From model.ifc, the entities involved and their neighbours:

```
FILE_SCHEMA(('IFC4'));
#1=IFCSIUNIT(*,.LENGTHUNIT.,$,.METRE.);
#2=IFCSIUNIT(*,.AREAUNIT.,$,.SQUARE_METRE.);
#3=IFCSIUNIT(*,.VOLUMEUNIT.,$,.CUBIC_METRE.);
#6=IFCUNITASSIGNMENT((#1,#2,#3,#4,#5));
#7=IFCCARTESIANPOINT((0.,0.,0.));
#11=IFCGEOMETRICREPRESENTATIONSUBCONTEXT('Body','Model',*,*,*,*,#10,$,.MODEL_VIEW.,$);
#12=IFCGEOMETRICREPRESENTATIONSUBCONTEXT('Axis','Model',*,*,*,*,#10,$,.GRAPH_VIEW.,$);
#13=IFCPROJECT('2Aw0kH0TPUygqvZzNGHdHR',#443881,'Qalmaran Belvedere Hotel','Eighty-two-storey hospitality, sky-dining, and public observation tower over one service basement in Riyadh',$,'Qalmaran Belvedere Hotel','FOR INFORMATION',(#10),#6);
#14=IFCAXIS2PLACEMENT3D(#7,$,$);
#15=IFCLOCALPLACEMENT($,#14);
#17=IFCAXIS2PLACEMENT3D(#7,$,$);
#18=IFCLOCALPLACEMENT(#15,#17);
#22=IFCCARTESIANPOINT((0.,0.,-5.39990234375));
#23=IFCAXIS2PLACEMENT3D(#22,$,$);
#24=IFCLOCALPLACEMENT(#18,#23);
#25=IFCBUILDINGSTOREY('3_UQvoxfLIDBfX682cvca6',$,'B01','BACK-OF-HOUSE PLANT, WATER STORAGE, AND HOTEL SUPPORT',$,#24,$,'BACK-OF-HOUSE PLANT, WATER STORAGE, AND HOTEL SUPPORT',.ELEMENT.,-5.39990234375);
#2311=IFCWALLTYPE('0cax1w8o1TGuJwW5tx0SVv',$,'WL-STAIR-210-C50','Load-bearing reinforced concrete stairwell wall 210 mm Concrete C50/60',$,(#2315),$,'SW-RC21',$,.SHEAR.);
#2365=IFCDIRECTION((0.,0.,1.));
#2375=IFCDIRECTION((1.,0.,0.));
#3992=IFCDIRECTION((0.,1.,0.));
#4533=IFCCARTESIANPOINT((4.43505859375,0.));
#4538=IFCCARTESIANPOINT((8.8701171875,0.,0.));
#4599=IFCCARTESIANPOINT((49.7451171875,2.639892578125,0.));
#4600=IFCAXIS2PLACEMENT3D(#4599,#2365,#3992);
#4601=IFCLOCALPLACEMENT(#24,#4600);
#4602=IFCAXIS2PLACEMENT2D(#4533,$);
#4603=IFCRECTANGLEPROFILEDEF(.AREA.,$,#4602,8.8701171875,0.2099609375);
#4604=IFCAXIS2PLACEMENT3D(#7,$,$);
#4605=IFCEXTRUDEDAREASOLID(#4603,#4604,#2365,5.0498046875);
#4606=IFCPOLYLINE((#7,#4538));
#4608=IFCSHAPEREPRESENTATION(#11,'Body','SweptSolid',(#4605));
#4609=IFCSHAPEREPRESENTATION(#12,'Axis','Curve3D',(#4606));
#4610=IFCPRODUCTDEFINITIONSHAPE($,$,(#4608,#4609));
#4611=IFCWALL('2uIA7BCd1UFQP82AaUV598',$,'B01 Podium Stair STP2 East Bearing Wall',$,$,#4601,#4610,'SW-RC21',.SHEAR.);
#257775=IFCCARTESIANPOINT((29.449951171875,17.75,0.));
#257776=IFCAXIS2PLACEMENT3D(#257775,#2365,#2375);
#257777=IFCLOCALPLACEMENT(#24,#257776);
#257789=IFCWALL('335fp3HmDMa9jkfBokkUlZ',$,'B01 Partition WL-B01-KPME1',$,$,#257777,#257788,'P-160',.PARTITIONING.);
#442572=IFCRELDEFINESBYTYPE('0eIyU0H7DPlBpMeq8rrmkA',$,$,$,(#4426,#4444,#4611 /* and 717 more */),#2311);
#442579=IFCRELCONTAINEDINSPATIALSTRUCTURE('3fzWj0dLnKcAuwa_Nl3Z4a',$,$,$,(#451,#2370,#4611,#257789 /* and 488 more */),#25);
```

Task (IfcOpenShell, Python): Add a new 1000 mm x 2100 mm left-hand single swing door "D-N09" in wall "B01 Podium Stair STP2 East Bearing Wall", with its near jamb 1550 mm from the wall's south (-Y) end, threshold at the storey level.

```python
import numpy as np
import ifcopenshell
import ifcopenshell.api.feature
import ifcopenshell.api.geometry
import ifcopenshell.api.root
import ifcopenshell.api.spatial
import ifcopenshell.geom
import ifcopenshell.util.element
import ifcopenshell.util.placement
import ifcopenshell.util.representation
import ifcopenshell.util.shape
import ifcopenshell.util.unit

model = ifcopenshell.open("model.ifc")
unit_scale = ifcopenshell.util.unit.calculate_unit_scale(model)
settings = ifcopenshell.geom.settings()


def volume(element):
    """Net volume in cubic metres, openings subtracted."""
    shape = ifcopenshell.geom.create_shape(settings, element)
    return ifcopenshell.util.shape.get_volume(shape.geometry)


wall = model.by_guid("2uIA7BCd1UFQP82AaUV598")
storey = ifcopenshell.util.element.get_container(wall, ifc_class="IfcBuildingStorey")
context = ifcopenshell.util.representation.get_context(model, "Model", "Body", "MODEL_VIEW")
before = volume(wall)

width, height, from_end, sill = 1, 2.1, 1.55, 0.0  # metres

# The wall runs along its own X axis, and the end named is its -X end.
wall_shape = ifcopenshell.geom.create_shape(settings, wall)
x, y, z = ifcopenshell.util.shape.get_vertices(wall_shape.geometry).T
start = x.min() + from_end
face, thickness = float(y.min()), float(y.max() - y.min())
wall_matrix = ifcopenshell.util.placement.get_local_placement(wall.ObjectPlacement)
level = ifcopenshell.util.placement.get_local_placement(storey.ObjectPlacement)[2, 3]


def in_wall(x, y):
    """Placement at x, y metres in the wall's axes, at sill height."""
    matrix = wall_matrix.copy()
    matrix[:, 3] = wall_matrix @ np.array([x / unit_scale, y / unit_scale, 0.0, 1.0])
    matrix[2, 3] = level + sill / unit_scale
    return matrix


# Opening: a box that overshoots both wall faces by 50 mm.
opening = ifcopenshell.api.root.create_entity(model, ifc_class="IfcOpeningElement", predefined_type="OPENING")
box = ifcopenshell.api.geometry.add_wall_representation(
    model, context=context, length=width, height=height, thickness=thickness + 0.1
)
ifcopenshell.api.geometry.assign_representation(model, product=opening, representation=box)
ifcopenshell.api.geometry.edit_object_placement(model, product=opening, matrix=in_wall(start, face - 0.05), is_si=False)
ifcopenshell.api.feature.add_feature(model, feature=opening, element=wall)

door = ifcopenshell.api.root.create_entity(model, ifc_class="IfcDoor", name="D-N09", predefined_type="DOOR")
door.OverallWidth, door.OverallHeight = width / unit_scale, height / unit_scale
door.OperationType = "SINGLE_SWING_LEFT"
body = ifcopenshell.api.geometry.add_door_representation(
    model,
    context=context,
    overall_width=door.OverallWidth,
    overall_height=door.OverallHeight,
    operation_type="SINGLE_SWING_LEFT",
    lining_properties={"LiningDepth": thickness / unit_scale, "ThresholdDepth": thickness / unit_scale},
)
ifcopenshell.api.geometry.assign_representation(model, product=door, representation=body)
ifcopenshell.api.spatial.assign_container(model, products=[door], relating_structure=storey)
ifcopenshell.api.feature.add_filling(model, opening=opening, element=door)

# The lining spans the wall, so the door starts at the wall face.
ifcopenshell.api.geometry.edit_object_placement(model, product=door, matrix=in_wall(start, face), is_si=False)

after = volume(wall)

print(f"wall volume {before:.3f} -> {after:.3f} m3")

model.write("model_rev.ifc")
```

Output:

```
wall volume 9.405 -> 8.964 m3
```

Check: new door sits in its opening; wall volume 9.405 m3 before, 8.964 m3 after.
